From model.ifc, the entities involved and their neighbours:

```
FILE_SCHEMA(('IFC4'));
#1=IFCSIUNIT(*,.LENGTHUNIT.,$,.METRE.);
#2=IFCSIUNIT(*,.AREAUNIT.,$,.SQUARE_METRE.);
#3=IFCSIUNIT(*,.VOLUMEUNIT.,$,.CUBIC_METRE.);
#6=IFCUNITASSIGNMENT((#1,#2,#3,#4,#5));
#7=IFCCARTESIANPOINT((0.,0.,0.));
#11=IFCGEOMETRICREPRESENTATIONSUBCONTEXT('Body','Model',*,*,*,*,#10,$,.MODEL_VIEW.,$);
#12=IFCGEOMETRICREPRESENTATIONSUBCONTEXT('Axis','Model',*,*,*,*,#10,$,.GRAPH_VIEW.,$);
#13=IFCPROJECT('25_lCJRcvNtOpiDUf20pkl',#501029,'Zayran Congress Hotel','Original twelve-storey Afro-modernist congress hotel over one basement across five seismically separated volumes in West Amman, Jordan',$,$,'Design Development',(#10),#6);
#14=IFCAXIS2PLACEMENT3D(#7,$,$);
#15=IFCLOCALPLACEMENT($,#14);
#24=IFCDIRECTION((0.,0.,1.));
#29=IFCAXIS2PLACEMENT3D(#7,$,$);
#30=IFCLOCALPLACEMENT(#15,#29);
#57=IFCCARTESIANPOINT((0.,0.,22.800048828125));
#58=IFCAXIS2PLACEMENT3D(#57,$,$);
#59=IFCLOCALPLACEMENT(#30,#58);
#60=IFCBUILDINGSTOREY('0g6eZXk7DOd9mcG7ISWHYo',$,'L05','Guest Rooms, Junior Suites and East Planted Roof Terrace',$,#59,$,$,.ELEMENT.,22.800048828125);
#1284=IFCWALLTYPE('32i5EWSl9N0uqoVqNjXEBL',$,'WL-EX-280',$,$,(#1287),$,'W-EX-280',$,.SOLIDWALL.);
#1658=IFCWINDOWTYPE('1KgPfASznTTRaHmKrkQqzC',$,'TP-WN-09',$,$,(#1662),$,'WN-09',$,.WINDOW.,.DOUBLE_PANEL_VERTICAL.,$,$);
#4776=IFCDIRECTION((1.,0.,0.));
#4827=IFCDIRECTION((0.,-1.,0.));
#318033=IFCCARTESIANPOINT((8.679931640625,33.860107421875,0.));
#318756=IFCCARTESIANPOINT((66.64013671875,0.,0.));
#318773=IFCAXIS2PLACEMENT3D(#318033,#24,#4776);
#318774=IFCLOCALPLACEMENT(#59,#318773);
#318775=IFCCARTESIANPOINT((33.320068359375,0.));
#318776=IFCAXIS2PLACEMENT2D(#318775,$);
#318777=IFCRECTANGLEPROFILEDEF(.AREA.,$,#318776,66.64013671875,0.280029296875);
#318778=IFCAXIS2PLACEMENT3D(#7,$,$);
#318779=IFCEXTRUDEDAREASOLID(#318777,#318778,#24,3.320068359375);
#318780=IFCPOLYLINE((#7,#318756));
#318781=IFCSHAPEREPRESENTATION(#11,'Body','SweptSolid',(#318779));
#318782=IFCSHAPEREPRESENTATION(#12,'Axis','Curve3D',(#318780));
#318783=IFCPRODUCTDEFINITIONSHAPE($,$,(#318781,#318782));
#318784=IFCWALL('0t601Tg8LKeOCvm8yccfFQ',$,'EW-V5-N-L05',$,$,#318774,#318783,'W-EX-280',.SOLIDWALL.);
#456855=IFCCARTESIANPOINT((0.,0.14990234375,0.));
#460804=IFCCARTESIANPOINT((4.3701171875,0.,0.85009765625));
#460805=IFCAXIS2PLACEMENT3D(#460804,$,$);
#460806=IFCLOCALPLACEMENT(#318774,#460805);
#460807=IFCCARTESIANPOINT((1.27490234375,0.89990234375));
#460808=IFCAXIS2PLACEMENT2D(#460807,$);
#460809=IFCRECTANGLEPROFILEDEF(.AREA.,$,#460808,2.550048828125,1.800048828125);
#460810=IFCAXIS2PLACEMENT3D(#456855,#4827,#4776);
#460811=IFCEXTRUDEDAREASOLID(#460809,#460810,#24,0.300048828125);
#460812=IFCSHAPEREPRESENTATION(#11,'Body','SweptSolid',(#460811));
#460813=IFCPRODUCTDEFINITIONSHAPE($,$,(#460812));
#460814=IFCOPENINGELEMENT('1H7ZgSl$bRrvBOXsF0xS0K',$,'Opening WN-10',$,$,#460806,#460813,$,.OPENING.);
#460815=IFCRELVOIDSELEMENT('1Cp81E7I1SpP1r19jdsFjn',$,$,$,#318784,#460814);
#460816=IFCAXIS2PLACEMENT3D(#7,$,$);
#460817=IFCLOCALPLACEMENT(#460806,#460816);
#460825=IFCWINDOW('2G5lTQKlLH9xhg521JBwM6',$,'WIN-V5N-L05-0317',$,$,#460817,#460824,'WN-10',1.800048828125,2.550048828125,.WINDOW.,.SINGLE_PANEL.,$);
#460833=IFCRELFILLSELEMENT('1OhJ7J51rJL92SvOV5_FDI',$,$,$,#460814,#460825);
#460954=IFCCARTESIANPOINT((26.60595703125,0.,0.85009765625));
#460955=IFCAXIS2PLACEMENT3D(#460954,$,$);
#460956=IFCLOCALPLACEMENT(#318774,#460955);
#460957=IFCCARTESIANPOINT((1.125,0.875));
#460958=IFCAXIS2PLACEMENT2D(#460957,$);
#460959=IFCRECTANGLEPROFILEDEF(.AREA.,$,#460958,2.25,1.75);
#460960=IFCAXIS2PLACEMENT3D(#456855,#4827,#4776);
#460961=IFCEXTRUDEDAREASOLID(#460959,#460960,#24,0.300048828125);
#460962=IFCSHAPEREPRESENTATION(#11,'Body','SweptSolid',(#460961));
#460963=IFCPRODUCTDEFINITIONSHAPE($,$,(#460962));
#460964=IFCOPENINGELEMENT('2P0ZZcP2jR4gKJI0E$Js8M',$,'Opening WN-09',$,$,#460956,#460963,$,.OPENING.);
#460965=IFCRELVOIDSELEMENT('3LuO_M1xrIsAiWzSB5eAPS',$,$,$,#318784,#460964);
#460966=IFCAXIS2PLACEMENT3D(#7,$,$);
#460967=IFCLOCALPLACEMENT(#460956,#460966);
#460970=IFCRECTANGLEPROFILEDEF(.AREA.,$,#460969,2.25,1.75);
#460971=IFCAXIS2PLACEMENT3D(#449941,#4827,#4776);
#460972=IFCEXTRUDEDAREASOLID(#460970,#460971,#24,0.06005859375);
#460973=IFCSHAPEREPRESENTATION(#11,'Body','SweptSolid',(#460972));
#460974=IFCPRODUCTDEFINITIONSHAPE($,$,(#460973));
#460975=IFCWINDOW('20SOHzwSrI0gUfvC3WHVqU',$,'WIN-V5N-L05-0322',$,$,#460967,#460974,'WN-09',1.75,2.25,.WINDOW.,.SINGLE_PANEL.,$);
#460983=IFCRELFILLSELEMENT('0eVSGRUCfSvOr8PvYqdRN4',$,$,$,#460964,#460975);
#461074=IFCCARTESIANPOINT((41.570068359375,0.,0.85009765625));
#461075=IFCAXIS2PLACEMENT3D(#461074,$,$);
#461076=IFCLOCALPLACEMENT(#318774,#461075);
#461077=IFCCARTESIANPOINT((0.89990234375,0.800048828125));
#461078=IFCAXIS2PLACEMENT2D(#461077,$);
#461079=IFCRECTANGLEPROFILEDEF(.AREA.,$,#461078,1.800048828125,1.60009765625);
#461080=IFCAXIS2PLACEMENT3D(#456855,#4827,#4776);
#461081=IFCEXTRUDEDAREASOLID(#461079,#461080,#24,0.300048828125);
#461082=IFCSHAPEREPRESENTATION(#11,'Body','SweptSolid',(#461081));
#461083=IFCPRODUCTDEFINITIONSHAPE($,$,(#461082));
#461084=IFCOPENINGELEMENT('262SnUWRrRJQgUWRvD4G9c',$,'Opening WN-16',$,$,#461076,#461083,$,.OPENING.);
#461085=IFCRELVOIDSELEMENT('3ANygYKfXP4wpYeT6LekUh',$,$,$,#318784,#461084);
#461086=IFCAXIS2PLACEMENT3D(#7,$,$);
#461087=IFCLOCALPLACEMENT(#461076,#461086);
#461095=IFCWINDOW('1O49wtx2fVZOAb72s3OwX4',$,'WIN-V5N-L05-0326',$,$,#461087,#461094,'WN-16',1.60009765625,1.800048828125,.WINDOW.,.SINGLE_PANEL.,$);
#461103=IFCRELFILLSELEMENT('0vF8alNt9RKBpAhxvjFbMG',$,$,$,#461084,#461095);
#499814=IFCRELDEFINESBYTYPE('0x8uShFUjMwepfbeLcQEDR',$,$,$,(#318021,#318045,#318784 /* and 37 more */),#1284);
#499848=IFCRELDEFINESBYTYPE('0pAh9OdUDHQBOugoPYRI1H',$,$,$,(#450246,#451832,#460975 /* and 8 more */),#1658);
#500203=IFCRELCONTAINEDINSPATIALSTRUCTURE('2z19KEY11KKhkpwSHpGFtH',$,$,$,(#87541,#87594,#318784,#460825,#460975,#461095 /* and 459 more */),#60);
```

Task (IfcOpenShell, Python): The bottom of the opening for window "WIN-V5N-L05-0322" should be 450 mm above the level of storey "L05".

```python
import numpy as np
import ifcopenshell
import ifcopenshell.api.geometry
import ifcopenshell.geom
import ifcopenshell.util.element
import ifcopenshell.util.placement
import ifcopenshell.util.shape
import ifcopenshell.util.unit

model = ifcopenshell.open("model.ifc")
unit_scale = ifcopenshell.util.unit.calculate_unit_scale(model)

window = model.by_guid("20SOHzwSrI0gUfvC3WHVqU")
opening = window.FillsVoids[0].RelatingOpeningElement
storey = ifcopenshell.util.element.get_container(window, ifc_class="IfcBuildingStorey")
level = ifcopenshell.util.placement.get_local_placement(storey.ObjectPlacement)[2, 3]

# The opening's origin need not be at the sill, so measure its lowest point.
shape = ifcopenshell.geom.create_shape(ifcopenshell.geom.settings(), opening)
bottom = ifcopenshell.util.shape.get_shape_bottom_elevation(shape, shape.geometry) / unit_scale
dz = level + 0.45 / unit_scale - bottom

shift = np.array([0.0, 0.0, dz])
# The window is placed relative to its opening, so it follows when the opening moves.
matrix = ifcopenshell.util.placement.get_local_placement(opening.ObjectPlacement)
matrix[:3, 3] += shift
ifcopenshell.api.geometry.edit_object_placement(
    model, product=opening, matrix=matrix, is_si=False, should_transform_children=True
)

print(f"moved by {dz * unit_scale:+.3f} m")

model.write("model-out.ifc")
```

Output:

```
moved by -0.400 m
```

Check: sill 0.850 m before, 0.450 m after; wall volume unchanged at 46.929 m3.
